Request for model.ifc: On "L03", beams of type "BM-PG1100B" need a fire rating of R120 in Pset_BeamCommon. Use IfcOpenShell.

First a look at what the model holds.

```python
import ifcopenshell
import ifcopenshell.util.element

model = ifcopenshell.open("model.ifc")
print(model.schema)
storey = next(s for s in model.by_type("IfcBuildingStorey") if s.Name == "L03")
beams = [e for e in ifcopenshell.util.element.get_decomposition(storey) if e.is_a("IfcBeam")]
seen = {}
for e in beams:
    element_type = ifcopenshell.util.element.get_type(e)
    key = (element_type.Name if element_type != e and element_type else None, ifcopenshell.util.element.get_pset(e, "Pset_BeamCommon", "FireRating"))
    seen[key] = seen.get(key, 0) + 1
for (name, value), count in sorted(seen.items(), key=str):
    print(count, "x", name, "|", value)
```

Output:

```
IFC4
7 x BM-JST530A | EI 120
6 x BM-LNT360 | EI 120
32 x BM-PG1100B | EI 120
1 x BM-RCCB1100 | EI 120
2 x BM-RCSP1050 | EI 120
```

```python
import ifcopenshell
import ifcopenshell.api.pset
import ifcopenshell.util.element

model = ifcopenshell.open("model.ifc")

storey = next(s for s in model.by_type("IfcBuildingStorey") if s.Name == "L03")
beams = [e for e in ifcopenshell.util.element.get_decomposition(storey) if e.is_a("IfcBeam")]

count = 0
for e in beams:
    element_type = ifcopenshell.util.element.get_type(e)
    if element_type in (None, e) or element_type.Name != "BM-PG1100B":
        continue
    found = ifcopenshell.util.element.get_pset(e, "Pset_BeamCommon", should_inherit=False)
    if found:
        pset = model.by_id(found["id"])
        if len(ifcopenshell.util.element.get_elements_by_pset(pset)) > 1:
            pset = ifcopenshell.api.pset.unshare_pset(model, products=[e], pset=pset)[0]
    else:
        pset = ifcopenshell.api.pset.add_pset(model, product=e, name="Pset_BeamCommon")
    ifcopenshell.api.pset.edit_pset(model, pset=pset, properties={"FireRating": "R120"})
    count += 1

print(count, "beams updated")

model.write("model_v2.ifc")
```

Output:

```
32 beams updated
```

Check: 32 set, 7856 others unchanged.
